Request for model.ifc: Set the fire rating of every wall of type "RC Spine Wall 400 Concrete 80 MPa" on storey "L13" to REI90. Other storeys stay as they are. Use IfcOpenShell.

First a look at what the model holds.

```python
import ifcopenshell
import ifcopenshell.util.element

model = ifcopenshell.open("model.ifc")
print(model.schema)
storey = next(s for s in model.by_type("IfcBuildingStorey") if s.Name == "L13")
walls = [e for e in ifcopenshell.util.element.get_decomposition(storey) if e.is_a("IfcWall")]
seen = {}
for e in walls:
    element_type = ifcopenshell.util.element.get_type(e)
    key = (element_type.Name if element_type != e and element_type else None, ifcopenshell.util.element.get_pset(e, "Pset_WallCommon", "FireRating"))
    seen[key] = seen.get(key, 0) + 1
for (name, value), count in sorted(seen.items(), key=str):
    print(count, "x", name, "|", value)
```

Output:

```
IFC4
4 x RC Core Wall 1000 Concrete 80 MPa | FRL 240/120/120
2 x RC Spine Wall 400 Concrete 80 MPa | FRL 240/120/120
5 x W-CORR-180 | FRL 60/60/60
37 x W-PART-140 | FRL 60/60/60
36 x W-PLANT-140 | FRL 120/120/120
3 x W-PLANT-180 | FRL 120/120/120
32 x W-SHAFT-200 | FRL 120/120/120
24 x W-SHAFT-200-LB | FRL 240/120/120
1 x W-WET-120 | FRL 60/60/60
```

```python
import ifcopenshell
import ifcopenshell.api.pset
import ifcopenshell.util.element

model = ifcopenshell.open("model.ifc")

storey = next(s for s in model.by_type("IfcBuildingStorey") if s.Name == "L13")
walls = [e for e in ifcopenshell.util.element.get_decomposition(storey) if e.is_a("IfcWall")]

count = 0
for e in walls:
    element_type = ifcopenshell.util.element.get_type(e)
    if element_type in (None, e) or element_type.Name != "RC Spine Wall 400 Concrete 80 MPa":
        continue
    # add_pset returns the element's existing set when there is one.
    pset = ifcopenshell.api.pset.add_pset(model, product=e, name="Pset_WallCommon")
    ifcopenshell.api.pset.edit_pset(model, pset=pset, properties={"FireRating": "REI90"})
    count += 1

print(count, "walls updated")

model.write("model_v2.ifc")
```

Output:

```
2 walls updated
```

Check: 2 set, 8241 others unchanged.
